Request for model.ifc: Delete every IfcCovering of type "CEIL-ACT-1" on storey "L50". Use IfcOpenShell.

First a look at what the model holds.

```python
import ifcopenshell
import ifcopenshell.util.element

model = ifcopenshell.open("model.ifc")
print(model.schema)
storey = next(s for s in model.by_type("IfcBuildingStorey") if s.Name == "L50")
coverings = [e for e in ifcopenshell.util.element.get_decomposition(storey) if e.is_a("IfcCovering")]
seen = {}
for e in coverings:
    element_type = ifcopenshell.util.element.get_type(e)
    name = element_type.Name if element_type not in (None, e) else None
    seen[name] = seen.get(name, 0) + 1
for name, count in sorted(seen.items(), key=str):
    print(count, "x", name)
```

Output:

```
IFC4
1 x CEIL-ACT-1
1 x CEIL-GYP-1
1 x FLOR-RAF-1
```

```python
import ifcopenshell
import ifcopenshell.api.root
import ifcopenshell.util.element

model = ifcopenshell.open("model.ifc")

storey = next(s for s in model.by_type("IfcBuildingStorey") if s.Name == "L50")
coverings = [e for e in ifcopenshell.util.element.get_decomposition(storey) if e.is_a("IfcCovering")]
targets = [e for e in coverings if (t := ifcopenshell.util.element.get_type(e)) not in (None, e) and t.Name == "CEIL-ACT-1"]

for e in targets:
    ifcopenshell.api.root.remove_product(model, product=e)
print(len(targets), "removed")

model.write("model-out.ifc")
```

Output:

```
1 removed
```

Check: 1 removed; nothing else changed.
